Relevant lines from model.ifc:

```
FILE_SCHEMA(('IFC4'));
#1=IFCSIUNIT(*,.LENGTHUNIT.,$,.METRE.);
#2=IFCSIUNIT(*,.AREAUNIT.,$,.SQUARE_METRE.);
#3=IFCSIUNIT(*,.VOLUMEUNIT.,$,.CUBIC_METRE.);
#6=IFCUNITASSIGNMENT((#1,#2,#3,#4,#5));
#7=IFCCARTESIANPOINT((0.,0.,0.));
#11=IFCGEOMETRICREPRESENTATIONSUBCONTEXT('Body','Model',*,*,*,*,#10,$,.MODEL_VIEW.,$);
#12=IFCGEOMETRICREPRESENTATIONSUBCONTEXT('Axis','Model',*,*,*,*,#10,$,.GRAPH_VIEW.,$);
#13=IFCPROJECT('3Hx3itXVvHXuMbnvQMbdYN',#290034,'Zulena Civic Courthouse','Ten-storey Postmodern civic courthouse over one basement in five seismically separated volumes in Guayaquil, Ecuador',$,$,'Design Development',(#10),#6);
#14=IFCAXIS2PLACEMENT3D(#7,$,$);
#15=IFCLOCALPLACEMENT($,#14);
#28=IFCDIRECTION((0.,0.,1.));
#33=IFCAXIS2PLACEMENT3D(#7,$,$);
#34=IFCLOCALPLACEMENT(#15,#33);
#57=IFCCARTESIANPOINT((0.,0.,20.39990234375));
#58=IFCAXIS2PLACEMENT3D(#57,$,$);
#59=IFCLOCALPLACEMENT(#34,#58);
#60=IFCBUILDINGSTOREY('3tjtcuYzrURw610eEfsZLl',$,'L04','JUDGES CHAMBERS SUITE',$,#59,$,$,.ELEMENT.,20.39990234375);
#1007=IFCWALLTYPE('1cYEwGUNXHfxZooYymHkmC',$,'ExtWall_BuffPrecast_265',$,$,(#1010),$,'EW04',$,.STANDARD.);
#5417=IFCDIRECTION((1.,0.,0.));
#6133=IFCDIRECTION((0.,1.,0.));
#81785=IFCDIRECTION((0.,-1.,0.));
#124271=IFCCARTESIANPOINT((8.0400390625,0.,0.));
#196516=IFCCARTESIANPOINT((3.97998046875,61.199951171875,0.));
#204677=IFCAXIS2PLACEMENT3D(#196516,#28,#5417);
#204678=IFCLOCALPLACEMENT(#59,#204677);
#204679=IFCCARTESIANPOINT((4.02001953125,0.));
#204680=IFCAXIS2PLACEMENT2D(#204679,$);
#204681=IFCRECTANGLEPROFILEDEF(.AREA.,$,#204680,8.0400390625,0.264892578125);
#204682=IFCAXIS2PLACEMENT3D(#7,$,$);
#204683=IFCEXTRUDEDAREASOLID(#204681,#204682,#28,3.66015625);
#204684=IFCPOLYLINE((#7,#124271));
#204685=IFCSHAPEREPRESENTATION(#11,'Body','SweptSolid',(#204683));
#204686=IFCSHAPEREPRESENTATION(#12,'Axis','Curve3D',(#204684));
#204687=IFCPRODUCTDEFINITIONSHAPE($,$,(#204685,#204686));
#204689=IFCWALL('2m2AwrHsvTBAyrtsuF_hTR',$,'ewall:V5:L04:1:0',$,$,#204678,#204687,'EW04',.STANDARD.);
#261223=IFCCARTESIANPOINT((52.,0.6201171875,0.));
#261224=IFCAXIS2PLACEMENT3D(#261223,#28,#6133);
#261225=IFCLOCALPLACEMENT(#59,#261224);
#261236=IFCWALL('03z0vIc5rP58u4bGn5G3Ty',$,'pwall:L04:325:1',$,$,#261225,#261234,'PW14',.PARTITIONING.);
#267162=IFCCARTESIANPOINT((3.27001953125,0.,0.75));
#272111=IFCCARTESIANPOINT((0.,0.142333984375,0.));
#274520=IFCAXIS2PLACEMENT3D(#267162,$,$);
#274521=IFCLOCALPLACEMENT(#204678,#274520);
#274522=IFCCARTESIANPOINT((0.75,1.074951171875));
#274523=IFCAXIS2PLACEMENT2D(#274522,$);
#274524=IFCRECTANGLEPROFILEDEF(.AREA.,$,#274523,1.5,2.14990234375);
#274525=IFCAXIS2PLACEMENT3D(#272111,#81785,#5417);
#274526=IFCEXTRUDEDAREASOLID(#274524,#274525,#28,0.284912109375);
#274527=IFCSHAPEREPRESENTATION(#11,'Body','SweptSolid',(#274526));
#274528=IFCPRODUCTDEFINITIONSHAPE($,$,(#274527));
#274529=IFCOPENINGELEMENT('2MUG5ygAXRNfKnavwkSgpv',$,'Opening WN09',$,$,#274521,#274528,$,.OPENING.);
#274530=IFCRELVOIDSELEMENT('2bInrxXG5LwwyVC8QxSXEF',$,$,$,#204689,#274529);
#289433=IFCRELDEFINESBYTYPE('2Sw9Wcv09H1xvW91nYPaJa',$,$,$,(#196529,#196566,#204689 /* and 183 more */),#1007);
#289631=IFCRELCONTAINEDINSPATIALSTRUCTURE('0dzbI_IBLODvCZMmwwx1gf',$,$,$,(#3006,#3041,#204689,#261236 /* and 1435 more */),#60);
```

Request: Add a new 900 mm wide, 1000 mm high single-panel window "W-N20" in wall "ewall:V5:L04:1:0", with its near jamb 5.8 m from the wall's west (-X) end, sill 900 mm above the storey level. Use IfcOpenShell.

```python
import numpy as np
import ifcopenshell
import ifcopenshell.api.feature
import ifcopenshell.api.geometry
import ifcopenshell.api.root
import ifcopenshell.api.spatial
import ifcopenshell.geom
import ifcopenshell.util.element
import ifcopenshell.util.placement
import ifcopenshell.util.representation
import ifcopenshell.util.shape
import ifcopenshell.util.unit

model = ifcopenshell.open("model.ifc")
unit_scale = ifcopenshell.util.unit.calculate_unit_scale(model)
settings = ifcopenshell.geom.settings()


def volume(element):
    """Net volume in cubic metres, openings subtracted."""
    shape = ifcopenshell.geom.create_shape(settings, element)
    return ifcopenshell.util.shape.get_volume(shape.geometry)


wall = model.by_guid("2m2AwrHsvTBAyrtsuF_hTR")
storey = ifcopenshell.util.element.get_container(wall, ifc_class="IfcBuildingStorey")
context = ifcopenshell.util.representation.get_context(model, "Model", "Body", "MODEL_VIEW")
before = volume(wall)

width, height, from_end, sill = 0.9, 1, 5.8, 0.9  # metres

# The wall runs along its own X axis, and the end named is its -X end.
wall_shape = ifcopenshell.geom.create_shape(settings, wall)
x, y, z = ifcopenshell.util.shape.get_vertices(wall_shape.geometry).T
start = x.min() + from_end
face, thickness = float(y.min()), float(y.max() - y.min())
wall_matrix = ifcopenshell.util.placement.get_local_placement(wall.ObjectPlacement)
level = ifcopenshell.util.placement.get_local_placement(storey.ObjectPlacement)[2, 3]


def in_wall(x, y):
    """Placement at x, y metres in the wall's axes, at sill height."""
    matrix = wall_matrix.copy()
    matrix[:, 3] = wall_matrix @ np.array([x / unit_scale, y / unit_scale, 0.0, 1.0])
    matrix[2, 3] = level + sill / unit_scale
    return matrix


# Opening: a box that overshoots both wall faces by 50 mm.
opening = ifcopenshell.api.root.create_entity(model, ifc_class="IfcOpeningElement", predefined_type="OPENING")
box = ifcopenshell.api.geometry.add_wall_representation(
    model, context=context, length=width, height=height, thickness=thickness + 0.1
)
ifcopenshell.api.geometry.assign_representation(model, product=opening, representation=box)
ifcopenshell.api.geometry.edit_object_placement(model, product=opening, matrix=in_wall(start, face - 0.05), is_si=False)
ifcopenshell.api.feature.add_feature(model, feature=opening, element=wall)

window = ifcopenshell.api.root.create_entity(model, ifc_class="IfcWindow", name="W-N20", predefined_type="WINDOW")
window.OverallWidth, window.OverallHeight = width / unit_scale, height / unit_scale
window.PartitioningType = "SINGLE_PANEL"
body = ifcopenshell.api.geometry.add_window_representation(
    model,
    context=context,
    overall_width=window.OverallWidth,
    overall_height=window.OverallHeight,
    partition_type="SINGLE_PANEL",
)
ifcopenshell.api.geometry.assign_representation(model, product=window, representation=body)
ifcopenshell.api.spatial.assign_container(model, products=[window], relating_structure=storey)
ifcopenshell.api.feature.add_filling(model, opening=opening, element=window)

# Centre the window in the wall's thickness.
ifcopenshell.api.geometry.edit_object_placement(model, product=window, matrix=in_wall(start, face), is_si=False)
window_shape = ifcopenshell.geom.create_shape(settings, window)
depth = ifcopenshell.util.shape.get_vertices(window_shape.geometry)[:, 1]
offset = face + thickness / 2 - (depth.min() + depth.max()) / 2
ifcopenshell.api.geometry.edit_object_placement(model, product=window, matrix=in_wall(start, offset), is_si=False)

after = volume(wall)

print(f"wall volume {before:.3f} -> {after:.3f} m3")

model.write("model_v2.ifc")
```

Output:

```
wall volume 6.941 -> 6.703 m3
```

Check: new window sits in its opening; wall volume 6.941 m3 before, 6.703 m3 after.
